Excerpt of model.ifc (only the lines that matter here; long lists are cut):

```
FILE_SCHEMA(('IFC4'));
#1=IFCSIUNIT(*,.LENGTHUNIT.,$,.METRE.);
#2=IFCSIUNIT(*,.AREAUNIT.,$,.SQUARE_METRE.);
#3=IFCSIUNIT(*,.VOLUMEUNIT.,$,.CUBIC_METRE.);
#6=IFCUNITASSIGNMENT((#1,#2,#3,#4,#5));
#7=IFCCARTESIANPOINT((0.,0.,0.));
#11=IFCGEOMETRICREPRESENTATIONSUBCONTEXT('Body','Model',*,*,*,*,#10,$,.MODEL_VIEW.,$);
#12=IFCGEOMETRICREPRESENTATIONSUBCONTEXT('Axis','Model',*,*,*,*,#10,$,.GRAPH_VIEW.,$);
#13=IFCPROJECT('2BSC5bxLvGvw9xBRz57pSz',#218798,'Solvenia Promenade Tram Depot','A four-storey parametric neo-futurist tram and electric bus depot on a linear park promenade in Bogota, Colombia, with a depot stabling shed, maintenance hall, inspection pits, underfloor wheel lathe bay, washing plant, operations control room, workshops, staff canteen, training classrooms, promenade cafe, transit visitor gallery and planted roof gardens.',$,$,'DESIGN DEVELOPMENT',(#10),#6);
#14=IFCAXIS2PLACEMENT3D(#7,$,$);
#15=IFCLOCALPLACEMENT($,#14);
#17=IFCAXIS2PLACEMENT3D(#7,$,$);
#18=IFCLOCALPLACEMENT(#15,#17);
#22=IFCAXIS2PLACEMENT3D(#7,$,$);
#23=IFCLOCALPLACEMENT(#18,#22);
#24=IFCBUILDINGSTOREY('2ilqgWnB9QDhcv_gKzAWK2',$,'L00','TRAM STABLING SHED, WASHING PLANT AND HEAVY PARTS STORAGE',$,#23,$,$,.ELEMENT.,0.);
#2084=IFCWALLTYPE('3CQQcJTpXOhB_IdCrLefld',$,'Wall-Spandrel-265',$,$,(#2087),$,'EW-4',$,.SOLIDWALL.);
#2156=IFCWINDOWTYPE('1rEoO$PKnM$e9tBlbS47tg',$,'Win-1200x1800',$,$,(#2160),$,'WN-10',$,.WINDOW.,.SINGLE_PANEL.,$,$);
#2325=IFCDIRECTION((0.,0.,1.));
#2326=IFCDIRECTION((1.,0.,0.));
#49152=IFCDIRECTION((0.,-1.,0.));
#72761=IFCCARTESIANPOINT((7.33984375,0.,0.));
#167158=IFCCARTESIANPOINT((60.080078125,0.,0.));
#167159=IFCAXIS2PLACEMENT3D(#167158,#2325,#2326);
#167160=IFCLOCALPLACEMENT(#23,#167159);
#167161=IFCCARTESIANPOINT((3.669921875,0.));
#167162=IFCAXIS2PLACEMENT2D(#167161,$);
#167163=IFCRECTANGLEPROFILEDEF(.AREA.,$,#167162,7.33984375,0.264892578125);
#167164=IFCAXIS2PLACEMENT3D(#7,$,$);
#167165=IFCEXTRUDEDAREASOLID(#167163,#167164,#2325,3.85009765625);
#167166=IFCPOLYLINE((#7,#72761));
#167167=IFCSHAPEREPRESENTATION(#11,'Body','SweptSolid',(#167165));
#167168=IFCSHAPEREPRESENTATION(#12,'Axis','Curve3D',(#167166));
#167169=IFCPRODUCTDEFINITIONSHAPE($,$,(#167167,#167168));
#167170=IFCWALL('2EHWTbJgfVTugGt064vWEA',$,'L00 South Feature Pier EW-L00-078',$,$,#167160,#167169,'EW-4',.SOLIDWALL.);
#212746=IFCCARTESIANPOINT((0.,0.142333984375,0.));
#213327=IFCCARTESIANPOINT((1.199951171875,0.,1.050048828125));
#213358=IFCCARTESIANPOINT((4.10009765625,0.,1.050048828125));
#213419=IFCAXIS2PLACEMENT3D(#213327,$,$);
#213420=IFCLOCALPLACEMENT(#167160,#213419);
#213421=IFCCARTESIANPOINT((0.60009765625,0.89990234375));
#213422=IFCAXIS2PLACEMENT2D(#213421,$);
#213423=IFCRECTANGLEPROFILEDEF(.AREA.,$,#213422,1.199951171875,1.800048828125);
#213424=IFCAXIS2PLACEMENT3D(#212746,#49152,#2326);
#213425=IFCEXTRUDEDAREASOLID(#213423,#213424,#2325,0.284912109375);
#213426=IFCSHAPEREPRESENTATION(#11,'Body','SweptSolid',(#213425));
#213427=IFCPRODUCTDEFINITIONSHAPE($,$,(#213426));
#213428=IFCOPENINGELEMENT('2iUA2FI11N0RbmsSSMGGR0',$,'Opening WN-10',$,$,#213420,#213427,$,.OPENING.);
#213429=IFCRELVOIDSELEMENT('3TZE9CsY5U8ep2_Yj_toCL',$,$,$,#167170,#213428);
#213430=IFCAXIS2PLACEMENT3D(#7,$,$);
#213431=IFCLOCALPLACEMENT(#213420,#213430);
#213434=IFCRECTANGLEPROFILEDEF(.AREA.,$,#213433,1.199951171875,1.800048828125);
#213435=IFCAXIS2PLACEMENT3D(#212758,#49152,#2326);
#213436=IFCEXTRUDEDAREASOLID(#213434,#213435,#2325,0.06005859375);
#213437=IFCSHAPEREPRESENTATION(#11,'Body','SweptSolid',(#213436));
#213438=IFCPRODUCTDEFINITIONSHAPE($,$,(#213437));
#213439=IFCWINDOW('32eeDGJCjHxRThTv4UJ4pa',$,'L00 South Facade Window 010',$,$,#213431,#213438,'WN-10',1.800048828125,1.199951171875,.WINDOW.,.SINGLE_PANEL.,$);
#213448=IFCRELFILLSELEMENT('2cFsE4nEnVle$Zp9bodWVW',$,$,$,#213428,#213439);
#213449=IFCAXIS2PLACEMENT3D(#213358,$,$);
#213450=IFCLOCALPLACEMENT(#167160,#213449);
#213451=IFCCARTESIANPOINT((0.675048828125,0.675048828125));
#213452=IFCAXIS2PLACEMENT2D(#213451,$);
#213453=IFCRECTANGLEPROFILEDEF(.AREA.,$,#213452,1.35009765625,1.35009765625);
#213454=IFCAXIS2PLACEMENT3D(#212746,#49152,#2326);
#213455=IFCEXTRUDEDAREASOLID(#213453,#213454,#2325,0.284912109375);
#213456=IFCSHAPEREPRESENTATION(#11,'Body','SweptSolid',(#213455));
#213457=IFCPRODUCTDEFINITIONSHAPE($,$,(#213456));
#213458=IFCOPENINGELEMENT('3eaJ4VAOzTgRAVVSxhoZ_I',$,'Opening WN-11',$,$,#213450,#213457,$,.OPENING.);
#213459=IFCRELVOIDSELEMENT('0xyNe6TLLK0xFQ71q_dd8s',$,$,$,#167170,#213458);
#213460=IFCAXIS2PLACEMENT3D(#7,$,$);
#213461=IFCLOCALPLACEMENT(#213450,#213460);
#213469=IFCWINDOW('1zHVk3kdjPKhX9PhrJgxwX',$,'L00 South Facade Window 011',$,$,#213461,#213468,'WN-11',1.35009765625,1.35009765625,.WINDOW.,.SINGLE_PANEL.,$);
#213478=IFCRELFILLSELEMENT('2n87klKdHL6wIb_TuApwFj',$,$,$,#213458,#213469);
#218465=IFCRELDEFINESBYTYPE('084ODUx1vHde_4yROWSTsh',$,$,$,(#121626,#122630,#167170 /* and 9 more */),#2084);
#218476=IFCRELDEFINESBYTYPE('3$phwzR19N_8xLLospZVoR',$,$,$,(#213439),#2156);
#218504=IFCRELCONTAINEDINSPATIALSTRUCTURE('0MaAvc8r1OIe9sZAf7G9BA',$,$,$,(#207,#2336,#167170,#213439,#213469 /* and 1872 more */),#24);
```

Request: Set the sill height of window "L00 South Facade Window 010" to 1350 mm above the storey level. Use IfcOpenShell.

```python
import numpy as np
import ifcopenshell
import ifcopenshell.api.geometry
import ifcopenshell.geom
import ifcopenshell.util.element
import ifcopenshell.util.placement
import ifcopenshell.util.shape
import ifcopenshell.util.unit

model = ifcopenshell.open("model.ifc")
unit_scale = ifcopenshell.util.unit.calculate_unit_scale(model)

window = model.by_guid("32eeDGJCjHxRThTv4UJ4pa")
opening = window.FillsVoids[0].RelatingOpeningElement
storey = ifcopenshell.util.element.get_container(window, ifc_class="IfcBuildingStorey")
level = ifcopenshell.util.placement.get_local_placement(storey.ObjectPlacement)[2, 3]

# The opening's origin need not be at the sill, so measure its lowest point.
shape = ifcopenshell.geom.create_shape(ifcopenshell.geom.settings(), opening)
bottom = ifcopenshell.util.shape.get_shape_bottom_elevation(shape, shape.geometry) / unit_scale
dz = level + 1.35 / unit_scale - bottom

shift = np.array([0.0, 0.0, dz])
# The window is placed relative to its opening, so it follows when the opening moves.
matrix = ifcopenshell.util.placement.get_local_placement(opening.ObjectPlacement)
matrix[:3, 3] += shift
ifcopenshell.api.geometry.edit_object_placement(
    model, product=opening, matrix=matrix, is_si=False, should_transform_children=True
)

print(f"moved by {dz * unit_scale:+.3f} m")

model.write("model_updated.ifc")
```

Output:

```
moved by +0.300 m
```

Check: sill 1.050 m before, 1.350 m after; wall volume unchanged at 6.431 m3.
